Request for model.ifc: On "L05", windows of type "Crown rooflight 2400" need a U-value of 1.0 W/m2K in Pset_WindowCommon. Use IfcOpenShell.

First a look at what the model holds.

```python
import ifcopenshell
import ifcopenshell.util.element

model = ifcopenshell.open("model.ifc")
print(model.schema)
storey = next(s for s in model.by_type("IfcBuildingStorey") if s.Name == "L05")
windows = [e for e in ifcopenshell.util.element.get_decomposition(storey) if e.is_a("IfcWindow")]
seen = {}
for e in windows:
    element_type = ifcopenshell.util.element.get_type(e)
    key = (element_type.Name if element_type != e and element_type else None, ifcopenshell.util.element.get_pset(e, "Pset_WindowCommon", "ThermalTransmittance"))
    seen[key] = seen.get(key, 0) + 1
for (name, value), count in sorted(seen.items(), key=str):
    print(count, "x", name, "|", value)
```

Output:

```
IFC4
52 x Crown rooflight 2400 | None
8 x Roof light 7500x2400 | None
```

```python
import ifcopenshell
import ifcopenshell.api.pset
import ifcopenshell.util.element

model = ifcopenshell.open("model.ifc")

storey = next(s for s in model.by_type("IfcBuildingStorey") if s.Name == "L05")
windows = [e for e in ifcopenshell.util.element.get_decomposition(storey) if e.is_a("IfcWindow")]

count = 0
for e in windows:
    element_type = ifcopenshell.util.element.get_type(e)
    if element_type in (None, e) or element_type.Name != "Crown rooflight 2400":
        continue
    # add_pset returns the element's existing set when there is one.
    pset = ifcopenshell.api.pset.add_pset(model, product=e, name="Pset_WindowCommon")
    ifcopenshell.api.pset.edit_pset(model, pset=pset, properties={"ThermalTransmittance": 1.0})
    count += 1

print(count, "windows updated")

model.write("model_v2.ifc")
```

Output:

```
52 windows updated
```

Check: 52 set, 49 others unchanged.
